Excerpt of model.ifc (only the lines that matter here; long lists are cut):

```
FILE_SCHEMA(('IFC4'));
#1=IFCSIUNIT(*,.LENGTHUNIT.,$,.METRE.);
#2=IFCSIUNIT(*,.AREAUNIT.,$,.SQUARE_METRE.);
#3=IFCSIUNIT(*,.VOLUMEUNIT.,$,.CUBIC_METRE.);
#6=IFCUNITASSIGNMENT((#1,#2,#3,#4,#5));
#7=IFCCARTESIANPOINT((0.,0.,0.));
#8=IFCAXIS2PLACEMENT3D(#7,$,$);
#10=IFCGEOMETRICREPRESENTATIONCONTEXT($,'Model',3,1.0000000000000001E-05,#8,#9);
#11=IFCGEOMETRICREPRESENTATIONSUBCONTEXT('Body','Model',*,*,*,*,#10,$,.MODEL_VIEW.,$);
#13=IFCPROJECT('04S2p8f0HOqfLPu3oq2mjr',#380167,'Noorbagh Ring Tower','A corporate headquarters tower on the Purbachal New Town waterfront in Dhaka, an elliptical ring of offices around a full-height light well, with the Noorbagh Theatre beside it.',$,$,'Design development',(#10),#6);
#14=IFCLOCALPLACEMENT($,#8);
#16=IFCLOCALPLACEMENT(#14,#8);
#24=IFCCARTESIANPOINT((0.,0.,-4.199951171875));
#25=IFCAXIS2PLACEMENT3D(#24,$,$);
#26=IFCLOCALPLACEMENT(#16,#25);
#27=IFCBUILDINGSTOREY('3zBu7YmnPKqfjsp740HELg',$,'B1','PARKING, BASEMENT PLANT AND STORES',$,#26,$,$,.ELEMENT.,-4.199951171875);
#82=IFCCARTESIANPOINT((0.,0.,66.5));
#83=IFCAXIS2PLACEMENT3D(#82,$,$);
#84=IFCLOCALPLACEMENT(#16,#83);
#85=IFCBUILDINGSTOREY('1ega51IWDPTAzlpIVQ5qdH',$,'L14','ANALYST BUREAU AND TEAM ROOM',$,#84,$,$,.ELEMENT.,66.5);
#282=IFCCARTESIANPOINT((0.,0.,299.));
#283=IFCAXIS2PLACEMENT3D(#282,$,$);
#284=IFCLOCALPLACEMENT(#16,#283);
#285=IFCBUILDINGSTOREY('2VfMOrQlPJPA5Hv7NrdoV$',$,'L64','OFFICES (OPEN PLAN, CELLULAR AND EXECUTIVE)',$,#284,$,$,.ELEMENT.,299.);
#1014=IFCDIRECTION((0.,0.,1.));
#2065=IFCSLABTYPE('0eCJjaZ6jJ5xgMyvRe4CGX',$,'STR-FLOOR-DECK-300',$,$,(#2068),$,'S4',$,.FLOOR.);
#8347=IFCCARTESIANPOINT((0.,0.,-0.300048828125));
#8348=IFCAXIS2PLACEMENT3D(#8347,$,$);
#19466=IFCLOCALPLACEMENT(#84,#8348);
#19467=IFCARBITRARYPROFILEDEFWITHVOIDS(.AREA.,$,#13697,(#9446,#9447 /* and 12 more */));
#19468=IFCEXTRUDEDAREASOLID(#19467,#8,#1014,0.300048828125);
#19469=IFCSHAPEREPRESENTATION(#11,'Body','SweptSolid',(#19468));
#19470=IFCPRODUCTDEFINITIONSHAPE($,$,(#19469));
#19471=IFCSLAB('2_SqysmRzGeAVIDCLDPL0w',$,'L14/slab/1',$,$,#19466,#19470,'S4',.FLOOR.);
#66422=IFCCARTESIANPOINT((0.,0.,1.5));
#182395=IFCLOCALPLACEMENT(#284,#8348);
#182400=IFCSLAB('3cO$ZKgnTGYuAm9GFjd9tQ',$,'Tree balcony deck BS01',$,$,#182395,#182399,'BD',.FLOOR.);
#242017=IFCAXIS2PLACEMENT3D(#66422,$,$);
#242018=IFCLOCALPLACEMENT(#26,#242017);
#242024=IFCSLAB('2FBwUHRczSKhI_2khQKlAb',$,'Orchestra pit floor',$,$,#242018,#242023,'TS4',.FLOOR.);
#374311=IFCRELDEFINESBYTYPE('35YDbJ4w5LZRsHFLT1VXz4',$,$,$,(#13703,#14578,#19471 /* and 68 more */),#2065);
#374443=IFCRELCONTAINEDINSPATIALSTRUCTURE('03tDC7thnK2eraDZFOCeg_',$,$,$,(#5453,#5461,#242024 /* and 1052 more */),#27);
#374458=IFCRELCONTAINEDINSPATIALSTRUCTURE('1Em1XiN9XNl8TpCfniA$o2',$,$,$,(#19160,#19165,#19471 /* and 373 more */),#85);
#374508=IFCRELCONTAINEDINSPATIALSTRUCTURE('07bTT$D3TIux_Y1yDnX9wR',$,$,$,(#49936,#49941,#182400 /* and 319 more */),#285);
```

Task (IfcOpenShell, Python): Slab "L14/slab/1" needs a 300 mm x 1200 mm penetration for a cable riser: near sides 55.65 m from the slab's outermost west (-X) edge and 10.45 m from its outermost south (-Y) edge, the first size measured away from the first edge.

```python
import numpy as np
import ifcopenshell
import ifcopenshell.api.feature
import ifcopenshell.api.geometry
import ifcopenshell.api.root
import ifcopenshell.geom
import ifcopenshell.util.placement
import ifcopenshell.util.representation
import ifcopenshell.util.shape
import ifcopenshell.util.unit

model = ifcopenshell.open("model.ifc")
unit_scale = ifcopenshell.util.unit.calculate_unit_scale(model)
settings = ifcopenshell.geom.settings()


def volume(element):
    """Net volume in cubic metres, openings subtracted."""
    shape = ifcopenshell.geom.create_shape(settings, element)
    return ifcopenshell.util.shape.get_volume(shape.geometry)


slab = model.by_guid("2_SqysmRzGeAVIDCLDPL0w")
before = volume(slab)

# Extent in the slab's own axes, in metres. The edges named are its -X and -Y sides.
slab_shape = ifcopenshell.geom.create_shape(settings, slab)
vertices = ifcopenshell.util.shape.get_vertices(slab_shape.geometry)
x_min, y_min, bottom = vertices.min(axis=0)
top = vertices[:, 2].max()

opening = ifcopenshell.api.root.create_entity(model, ifc_class="IfcOpeningElement", name="Cable riser opening", predefined_type="OPENING")
context = ifcopenshell.util.representation.get_context(model, "Model", "Body", "MODEL_VIEW")
width, depth = 0.3, 1.2
outline = [(0.0, 0.0), (width, 0.0), (width, depth), (0.0, depth), (0.0, 0.0)]
# Overshoot both faces by 50 mm so the cut is clean.
shape = ifcopenshell.api.geometry.add_slab_representation(
    model, context=context, depth=top - bottom + 0.1, polyline=outline
)
ifcopenshell.api.geometry.assign_representation(model, product=opening, representation=shape)

matrix = ifcopenshell.util.placement.get_local_placement(slab.ObjectPlacement)
matrix[:, 3] = matrix @ np.append(np.array([x_min + 55.65, y_min + 10.45, bottom - 0.05]) / unit_scale, 1.0)
ifcopenshell.api.geometry.edit_object_placement(model, product=opening, matrix=matrix, is_si=False)
ifcopenshell.api.feature.add_feature(model, feature=opening, element=slab)

after = volume(slab)

print(f"slab volume {before:.3f} -> {after:.3f} m3")

model.write("model_v2.ifc")
```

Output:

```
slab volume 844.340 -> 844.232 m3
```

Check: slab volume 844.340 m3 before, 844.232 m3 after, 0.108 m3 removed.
